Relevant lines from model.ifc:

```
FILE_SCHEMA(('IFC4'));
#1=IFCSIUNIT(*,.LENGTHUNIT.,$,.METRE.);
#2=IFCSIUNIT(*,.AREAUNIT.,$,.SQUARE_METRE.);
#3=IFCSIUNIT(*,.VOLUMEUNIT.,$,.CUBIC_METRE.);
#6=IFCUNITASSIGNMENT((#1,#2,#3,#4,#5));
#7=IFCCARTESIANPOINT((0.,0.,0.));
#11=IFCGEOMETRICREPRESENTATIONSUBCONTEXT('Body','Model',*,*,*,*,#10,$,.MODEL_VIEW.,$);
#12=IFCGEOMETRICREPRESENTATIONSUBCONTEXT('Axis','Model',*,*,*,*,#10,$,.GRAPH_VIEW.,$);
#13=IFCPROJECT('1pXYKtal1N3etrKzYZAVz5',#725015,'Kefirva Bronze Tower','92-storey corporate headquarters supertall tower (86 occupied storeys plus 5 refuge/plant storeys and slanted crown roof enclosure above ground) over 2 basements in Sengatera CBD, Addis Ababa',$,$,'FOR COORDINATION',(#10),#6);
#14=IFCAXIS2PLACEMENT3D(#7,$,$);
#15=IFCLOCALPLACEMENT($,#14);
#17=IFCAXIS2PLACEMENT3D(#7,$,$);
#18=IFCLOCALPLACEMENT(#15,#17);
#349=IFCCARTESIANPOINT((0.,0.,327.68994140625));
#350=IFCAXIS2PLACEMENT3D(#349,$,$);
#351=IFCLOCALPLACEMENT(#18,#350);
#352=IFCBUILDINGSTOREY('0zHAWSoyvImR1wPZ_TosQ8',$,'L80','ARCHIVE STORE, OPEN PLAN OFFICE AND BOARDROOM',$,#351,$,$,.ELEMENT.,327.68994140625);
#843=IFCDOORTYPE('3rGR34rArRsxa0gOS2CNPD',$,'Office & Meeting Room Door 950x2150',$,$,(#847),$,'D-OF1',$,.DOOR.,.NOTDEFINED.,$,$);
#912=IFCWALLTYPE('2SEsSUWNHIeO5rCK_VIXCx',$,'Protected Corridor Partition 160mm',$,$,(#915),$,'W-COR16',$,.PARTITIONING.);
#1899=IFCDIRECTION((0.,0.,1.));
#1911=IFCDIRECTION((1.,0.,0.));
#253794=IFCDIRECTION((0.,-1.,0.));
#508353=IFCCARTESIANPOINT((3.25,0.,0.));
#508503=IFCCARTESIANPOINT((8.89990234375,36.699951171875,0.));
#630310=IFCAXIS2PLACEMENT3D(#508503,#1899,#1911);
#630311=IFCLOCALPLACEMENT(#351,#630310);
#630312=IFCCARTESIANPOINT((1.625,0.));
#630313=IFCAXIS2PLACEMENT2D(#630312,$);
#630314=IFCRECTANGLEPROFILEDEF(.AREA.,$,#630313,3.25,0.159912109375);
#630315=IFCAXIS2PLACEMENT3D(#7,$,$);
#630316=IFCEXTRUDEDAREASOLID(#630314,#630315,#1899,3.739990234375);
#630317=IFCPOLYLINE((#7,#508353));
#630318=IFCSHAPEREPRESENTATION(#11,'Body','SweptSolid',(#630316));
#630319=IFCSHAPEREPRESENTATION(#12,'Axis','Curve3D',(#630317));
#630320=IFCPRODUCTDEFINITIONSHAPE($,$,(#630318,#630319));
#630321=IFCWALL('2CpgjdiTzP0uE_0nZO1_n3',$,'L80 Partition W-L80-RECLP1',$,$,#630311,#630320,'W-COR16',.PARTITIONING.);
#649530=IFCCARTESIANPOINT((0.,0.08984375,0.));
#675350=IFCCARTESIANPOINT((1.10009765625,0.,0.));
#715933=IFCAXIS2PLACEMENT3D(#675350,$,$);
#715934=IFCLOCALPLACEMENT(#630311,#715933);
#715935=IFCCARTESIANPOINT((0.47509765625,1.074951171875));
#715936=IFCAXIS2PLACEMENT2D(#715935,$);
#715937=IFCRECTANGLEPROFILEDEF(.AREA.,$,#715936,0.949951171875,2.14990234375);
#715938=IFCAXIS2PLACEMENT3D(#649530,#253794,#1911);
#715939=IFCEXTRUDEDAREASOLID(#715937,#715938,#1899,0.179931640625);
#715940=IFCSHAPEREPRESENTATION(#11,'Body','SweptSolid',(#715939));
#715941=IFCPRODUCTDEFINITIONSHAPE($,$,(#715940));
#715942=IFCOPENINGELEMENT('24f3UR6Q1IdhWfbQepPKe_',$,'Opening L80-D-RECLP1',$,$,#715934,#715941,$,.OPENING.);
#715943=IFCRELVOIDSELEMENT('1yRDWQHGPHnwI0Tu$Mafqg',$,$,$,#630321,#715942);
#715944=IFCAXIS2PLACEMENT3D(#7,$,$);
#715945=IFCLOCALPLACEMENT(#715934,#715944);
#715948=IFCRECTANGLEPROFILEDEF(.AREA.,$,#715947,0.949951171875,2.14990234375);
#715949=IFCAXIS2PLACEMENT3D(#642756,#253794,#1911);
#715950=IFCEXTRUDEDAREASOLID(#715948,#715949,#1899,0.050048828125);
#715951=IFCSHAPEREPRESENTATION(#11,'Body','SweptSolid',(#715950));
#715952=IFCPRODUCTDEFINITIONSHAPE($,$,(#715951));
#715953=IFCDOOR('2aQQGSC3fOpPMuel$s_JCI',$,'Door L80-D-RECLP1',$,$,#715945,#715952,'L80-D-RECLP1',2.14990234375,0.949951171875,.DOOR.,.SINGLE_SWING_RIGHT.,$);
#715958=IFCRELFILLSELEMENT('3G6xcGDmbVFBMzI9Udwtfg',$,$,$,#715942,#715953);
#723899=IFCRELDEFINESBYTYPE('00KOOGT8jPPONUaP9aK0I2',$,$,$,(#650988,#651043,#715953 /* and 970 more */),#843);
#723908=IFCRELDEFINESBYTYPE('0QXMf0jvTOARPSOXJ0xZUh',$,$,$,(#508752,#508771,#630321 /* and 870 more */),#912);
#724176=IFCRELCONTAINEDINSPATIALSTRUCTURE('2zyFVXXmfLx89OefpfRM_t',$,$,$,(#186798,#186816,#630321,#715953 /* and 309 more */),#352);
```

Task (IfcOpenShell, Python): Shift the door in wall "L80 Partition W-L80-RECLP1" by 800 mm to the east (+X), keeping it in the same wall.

```python
import ifcopenshell
import ifcopenshell.api.geometry
import ifcopenshell.util.placement

model = ifcopenshell.open("model.ifc")

door = model.by_guid("2aQQGSC3fOpPMuel$s_JCI")
opening = door.FillsVoids[0].RelatingOpeningElement
wall = opening.VoidsElements[0].RelatingBuildingElement

wall_matrix = ifcopenshell.util.placement.get_local_placement(wall.ObjectPlacement)
shift = wall_matrix[:3, 0] * 0.8
before = ifcopenshell.util.placement.get_local_placement(door.ObjectPlacement)[:3, 3].copy()

# The door is placed relative to its opening, so it follows when the opening moves.
matrix = ifcopenshell.util.placement.get_local_placement(opening.ObjectPlacement)
matrix[:3, 3] += shift
ifcopenshell.api.geometry.edit_object_placement(
    model, product=opening, matrix=matrix, is_si=False, should_transform_children=True
)

after = ifcopenshell.util.placement.get_local_placement(door.ObjectPlacement)[:3, 3]
print("door moved by", (after - before).round(3) + 0.0)

model.write("model-out.ifc")
```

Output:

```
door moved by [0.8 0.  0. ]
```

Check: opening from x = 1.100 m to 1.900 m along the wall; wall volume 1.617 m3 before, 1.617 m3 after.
